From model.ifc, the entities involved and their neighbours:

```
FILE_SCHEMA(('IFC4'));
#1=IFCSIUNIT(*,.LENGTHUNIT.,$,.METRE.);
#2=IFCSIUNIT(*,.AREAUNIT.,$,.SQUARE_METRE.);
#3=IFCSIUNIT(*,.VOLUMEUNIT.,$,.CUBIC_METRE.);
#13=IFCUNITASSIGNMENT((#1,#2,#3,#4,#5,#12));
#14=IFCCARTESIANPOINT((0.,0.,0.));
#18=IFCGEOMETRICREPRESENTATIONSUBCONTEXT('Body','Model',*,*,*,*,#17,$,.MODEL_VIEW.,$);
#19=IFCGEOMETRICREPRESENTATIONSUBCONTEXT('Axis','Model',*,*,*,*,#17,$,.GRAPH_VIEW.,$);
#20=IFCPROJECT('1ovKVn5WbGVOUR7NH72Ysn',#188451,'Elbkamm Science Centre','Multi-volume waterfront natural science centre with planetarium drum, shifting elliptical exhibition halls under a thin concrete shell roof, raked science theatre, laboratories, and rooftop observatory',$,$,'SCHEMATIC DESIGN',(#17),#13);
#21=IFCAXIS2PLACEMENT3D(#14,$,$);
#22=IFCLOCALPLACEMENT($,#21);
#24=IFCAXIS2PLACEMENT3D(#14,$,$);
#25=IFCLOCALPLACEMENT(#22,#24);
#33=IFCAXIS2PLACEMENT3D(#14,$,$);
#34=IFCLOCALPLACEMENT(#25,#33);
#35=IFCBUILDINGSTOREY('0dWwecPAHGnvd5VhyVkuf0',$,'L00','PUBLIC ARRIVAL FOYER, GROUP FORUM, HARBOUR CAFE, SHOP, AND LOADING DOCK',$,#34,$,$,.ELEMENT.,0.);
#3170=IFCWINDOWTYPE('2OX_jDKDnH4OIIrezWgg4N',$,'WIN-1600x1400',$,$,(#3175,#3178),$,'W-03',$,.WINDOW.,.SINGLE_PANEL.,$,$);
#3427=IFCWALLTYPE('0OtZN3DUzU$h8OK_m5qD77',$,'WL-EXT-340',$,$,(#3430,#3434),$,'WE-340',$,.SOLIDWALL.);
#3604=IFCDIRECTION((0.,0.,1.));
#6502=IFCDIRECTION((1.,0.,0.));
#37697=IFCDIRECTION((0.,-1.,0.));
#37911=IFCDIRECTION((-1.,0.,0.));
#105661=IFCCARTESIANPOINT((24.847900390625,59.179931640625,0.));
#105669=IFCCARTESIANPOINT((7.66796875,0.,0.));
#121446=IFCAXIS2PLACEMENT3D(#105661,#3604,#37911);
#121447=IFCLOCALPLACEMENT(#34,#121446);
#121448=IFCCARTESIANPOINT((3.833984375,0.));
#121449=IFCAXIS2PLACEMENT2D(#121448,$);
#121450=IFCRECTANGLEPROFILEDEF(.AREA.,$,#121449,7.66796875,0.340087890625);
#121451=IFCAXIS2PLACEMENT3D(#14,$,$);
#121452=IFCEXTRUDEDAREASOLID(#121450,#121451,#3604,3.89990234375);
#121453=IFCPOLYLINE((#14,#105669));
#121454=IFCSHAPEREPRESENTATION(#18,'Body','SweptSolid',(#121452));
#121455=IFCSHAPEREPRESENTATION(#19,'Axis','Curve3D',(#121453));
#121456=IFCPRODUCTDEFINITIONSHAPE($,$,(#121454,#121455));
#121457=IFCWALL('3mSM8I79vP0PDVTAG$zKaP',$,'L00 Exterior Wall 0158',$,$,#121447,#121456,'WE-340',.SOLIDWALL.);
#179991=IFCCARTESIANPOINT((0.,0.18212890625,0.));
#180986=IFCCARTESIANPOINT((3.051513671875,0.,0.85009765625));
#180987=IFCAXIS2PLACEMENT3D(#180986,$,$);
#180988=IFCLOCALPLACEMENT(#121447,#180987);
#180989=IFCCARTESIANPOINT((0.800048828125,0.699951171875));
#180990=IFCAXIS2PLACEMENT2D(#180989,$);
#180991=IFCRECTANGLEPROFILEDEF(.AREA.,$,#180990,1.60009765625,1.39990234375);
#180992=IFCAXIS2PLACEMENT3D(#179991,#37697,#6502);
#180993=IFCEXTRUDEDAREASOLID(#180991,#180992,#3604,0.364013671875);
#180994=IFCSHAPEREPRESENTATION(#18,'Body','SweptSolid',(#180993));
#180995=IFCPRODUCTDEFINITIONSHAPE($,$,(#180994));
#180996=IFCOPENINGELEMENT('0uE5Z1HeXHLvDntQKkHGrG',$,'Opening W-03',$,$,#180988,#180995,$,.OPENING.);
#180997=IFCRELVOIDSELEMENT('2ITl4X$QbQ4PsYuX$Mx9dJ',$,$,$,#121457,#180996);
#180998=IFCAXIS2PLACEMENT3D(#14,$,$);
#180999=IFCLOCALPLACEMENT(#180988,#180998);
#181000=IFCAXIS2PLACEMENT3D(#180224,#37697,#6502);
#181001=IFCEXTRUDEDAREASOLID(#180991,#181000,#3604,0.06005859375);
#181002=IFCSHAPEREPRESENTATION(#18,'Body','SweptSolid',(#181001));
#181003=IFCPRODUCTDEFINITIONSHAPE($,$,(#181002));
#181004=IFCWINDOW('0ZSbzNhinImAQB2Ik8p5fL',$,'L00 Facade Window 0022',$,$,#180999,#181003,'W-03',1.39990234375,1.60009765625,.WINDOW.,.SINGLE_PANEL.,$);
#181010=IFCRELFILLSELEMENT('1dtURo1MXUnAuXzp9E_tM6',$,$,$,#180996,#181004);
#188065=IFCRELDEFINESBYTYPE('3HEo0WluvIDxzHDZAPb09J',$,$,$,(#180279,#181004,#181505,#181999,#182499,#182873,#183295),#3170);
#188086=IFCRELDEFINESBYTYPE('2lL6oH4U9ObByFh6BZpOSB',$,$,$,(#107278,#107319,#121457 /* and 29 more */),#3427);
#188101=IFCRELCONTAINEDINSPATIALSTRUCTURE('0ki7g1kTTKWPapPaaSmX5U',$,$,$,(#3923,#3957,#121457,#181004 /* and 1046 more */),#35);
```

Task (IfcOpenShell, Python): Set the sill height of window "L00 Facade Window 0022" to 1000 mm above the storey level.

```python
import numpy as np
import ifcopenshell
import ifcopenshell.api.geometry
import ifcopenshell.geom
import ifcopenshell.util.element
import ifcopenshell.util.placement
import ifcopenshell.util.shape
import ifcopenshell.util.unit

model = ifcopenshell.open("model.ifc")
unit_scale = ifcopenshell.util.unit.calculate_unit_scale(model)

window = model.by_guid("0ZSbzNhinImAQB2Ik8p5fL")
opening = window.FillsVoids[0].RelatingOpeningElement
storey = ifcopenshell.util.element.get_container(window, ifc_class="IfcBuildingStorey")
level = ifcopenshell.util.placement.get_local_placement(storey.ObjectPlacement)[2, 3]

# The opening's origin need not be at the sill, so measure its lowest point.
shape = ifcopenshell.geom.create_shape(ifcopenshell.geom.settings(), opening)
bottom = ifcopenshell.util.shape.get_shape_bottom_elevation(shape, shape.geometry) / unit_scale
dz = level + 1 / unit_scale - bottom

shift = np.array([0.0, 0.0, dz])
# The window is placed relative to its opening, so it follows when the opening moves.
matrix = ifcopenshell.util.placement.get_local_placement(opening.ObjectPlacement)
matrix[:3, 3] += shift
ifcopenshell.api.geometry.edit_object_placement(
    model, product=opening, matrix=matrix, is_si=False, should_transform_children=True
)

print(f"moved by {dz * unit_scale:+.3f} m")

model.write("model_edited.ifc")
```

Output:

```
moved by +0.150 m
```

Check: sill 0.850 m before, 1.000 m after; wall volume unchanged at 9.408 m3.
